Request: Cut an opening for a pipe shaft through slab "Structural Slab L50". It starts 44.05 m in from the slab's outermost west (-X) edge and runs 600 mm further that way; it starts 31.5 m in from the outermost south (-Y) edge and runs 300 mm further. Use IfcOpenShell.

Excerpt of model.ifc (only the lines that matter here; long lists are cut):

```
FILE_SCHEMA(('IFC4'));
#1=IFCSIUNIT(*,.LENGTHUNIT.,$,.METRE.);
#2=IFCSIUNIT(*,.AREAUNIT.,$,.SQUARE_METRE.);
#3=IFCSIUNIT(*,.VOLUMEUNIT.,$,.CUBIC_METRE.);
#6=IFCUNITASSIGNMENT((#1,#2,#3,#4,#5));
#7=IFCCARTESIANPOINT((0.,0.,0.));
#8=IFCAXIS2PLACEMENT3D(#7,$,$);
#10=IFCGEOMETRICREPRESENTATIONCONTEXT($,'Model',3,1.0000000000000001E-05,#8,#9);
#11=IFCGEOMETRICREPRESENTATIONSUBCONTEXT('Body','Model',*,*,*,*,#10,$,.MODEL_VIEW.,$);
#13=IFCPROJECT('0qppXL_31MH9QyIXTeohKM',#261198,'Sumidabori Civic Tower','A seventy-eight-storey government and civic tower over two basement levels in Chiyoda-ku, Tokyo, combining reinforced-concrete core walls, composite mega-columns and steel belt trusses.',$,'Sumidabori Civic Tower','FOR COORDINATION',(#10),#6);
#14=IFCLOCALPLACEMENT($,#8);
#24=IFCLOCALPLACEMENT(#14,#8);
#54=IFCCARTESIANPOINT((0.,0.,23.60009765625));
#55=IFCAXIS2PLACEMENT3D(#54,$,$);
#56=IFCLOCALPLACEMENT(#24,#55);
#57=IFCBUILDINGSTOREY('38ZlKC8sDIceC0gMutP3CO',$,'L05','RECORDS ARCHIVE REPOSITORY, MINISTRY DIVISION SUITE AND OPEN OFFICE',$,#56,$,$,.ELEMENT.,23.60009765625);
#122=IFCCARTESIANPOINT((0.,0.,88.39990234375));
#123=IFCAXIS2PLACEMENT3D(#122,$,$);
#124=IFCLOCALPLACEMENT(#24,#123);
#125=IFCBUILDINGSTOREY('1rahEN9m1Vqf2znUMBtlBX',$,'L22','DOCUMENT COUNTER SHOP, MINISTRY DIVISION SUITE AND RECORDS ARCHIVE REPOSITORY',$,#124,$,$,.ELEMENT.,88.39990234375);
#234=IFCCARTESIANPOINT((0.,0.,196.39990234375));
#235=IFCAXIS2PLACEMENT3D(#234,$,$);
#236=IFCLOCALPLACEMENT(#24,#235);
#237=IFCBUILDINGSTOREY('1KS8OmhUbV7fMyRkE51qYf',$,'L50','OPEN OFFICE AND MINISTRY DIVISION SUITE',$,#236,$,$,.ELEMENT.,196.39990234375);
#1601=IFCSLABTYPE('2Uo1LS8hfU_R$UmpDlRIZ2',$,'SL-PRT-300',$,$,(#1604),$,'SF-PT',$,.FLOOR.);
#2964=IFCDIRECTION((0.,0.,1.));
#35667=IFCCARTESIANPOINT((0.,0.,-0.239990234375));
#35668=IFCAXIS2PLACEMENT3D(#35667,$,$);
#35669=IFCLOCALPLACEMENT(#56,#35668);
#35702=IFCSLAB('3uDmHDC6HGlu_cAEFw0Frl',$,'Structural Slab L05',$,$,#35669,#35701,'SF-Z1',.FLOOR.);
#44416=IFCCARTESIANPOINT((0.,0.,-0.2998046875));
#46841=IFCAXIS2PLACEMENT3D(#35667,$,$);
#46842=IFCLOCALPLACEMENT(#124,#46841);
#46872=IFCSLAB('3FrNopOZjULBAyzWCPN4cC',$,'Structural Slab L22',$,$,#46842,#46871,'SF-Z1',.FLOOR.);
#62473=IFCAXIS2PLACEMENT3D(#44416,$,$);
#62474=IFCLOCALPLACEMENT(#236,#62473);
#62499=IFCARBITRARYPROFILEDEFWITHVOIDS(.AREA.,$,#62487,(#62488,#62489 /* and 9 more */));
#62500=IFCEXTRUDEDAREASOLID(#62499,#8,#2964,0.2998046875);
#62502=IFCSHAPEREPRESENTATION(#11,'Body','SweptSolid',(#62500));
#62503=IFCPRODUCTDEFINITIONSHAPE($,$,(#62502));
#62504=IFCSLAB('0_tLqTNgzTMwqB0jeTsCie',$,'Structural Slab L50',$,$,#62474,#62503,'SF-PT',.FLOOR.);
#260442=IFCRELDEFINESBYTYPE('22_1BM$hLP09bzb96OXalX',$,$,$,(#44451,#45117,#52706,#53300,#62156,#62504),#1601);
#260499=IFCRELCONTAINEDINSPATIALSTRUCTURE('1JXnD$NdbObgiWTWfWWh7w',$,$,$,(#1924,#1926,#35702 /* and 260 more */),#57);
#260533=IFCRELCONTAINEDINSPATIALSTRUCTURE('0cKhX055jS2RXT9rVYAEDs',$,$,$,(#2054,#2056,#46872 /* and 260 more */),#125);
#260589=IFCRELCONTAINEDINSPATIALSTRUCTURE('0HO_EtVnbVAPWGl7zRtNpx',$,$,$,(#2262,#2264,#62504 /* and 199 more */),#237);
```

```python
import numpy as np
import ifcopenshell
import ifcopenshell.api.feature
import ifcopenshell.api.geometry
import ifcopenshell.api.root
import ifcopenshell.geom
import ifcopenshell.util.placement
import ifcopenshell.util.representation
import ifcopenshell.util.shape
import ifcopenshell.util.unit

model = ifcopenshell.open("model.ifc")
unit_scale = ifcopenshell.util.unit.calculate_unit_scale(model)
settings = ifcopenshell.geom.settings()


def volume(element):
    """Net volume in cubic metres, openings subtracted."""
    shape = ifcopenshell.geom.create_shape(settings, element)
    return ifcopenshell.util.shape.get_volume(shape.geometry)


slab = model.by_id(62504)
before = volume(slab)

# Extent in the slab's own axes, in metres. The edges named are its -X and -Y sides.
slab_shape = ifcopenshell.geom.create_shape(settings, slab)
vertices = ifcopenshell.util.shape.get_vertices(slab_shape.geometry)
x_min, y_min, bottom = vertices.min(axis=0)
top = vertices[:, 2].max()

opening = ifcopenshell.api.root.create_entity(model, ifc_class="IfcOpeningElement", name="Pipe shaft opening", predefined_type="OPENING")
context = ifcopenshell.util.representation.get_context(model, "Model", "Body", "MODEL_VIEW")
width, depth = 0.6, 0.3
outline = [(0.0, 0.0), (width, 0.0), (width, depth), (0.0, depth), (0.0, 0.0)]
# Overshoot both faces by 50 mm so the cut is clean.
shape = ifcopenshell.api.geometry.add_slab_representation(
    model, context=context, depth=top - bottom + 0.1, polyline=outline
)
ifcopenshell.api.geometry.assign_representation(model, product=opening, representation=shape)

matrix = ifcopenshell.util.placement.get_local_placement(slab.ObjectPlacement)
matrix[:, 3] = matrix @ np.append(np.array([x_min + 44.05, y_min + 31.5, bottom - 0.05]) / unit_scale, 1.0)
ifcopenshell.api.geometry.edit_object_placement(model, product=opening, matrix=matrix, is_si=False)
ifcopenshell.api.feature.add_feature(model, feature=opening, element=slab)

after = volume(slab)

print(f"slab volume {before:.3f} -> {after:.3f} m3")

model.write("model_v2.ifc")
```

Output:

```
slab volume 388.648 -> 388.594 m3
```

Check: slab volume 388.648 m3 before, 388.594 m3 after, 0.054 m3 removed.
